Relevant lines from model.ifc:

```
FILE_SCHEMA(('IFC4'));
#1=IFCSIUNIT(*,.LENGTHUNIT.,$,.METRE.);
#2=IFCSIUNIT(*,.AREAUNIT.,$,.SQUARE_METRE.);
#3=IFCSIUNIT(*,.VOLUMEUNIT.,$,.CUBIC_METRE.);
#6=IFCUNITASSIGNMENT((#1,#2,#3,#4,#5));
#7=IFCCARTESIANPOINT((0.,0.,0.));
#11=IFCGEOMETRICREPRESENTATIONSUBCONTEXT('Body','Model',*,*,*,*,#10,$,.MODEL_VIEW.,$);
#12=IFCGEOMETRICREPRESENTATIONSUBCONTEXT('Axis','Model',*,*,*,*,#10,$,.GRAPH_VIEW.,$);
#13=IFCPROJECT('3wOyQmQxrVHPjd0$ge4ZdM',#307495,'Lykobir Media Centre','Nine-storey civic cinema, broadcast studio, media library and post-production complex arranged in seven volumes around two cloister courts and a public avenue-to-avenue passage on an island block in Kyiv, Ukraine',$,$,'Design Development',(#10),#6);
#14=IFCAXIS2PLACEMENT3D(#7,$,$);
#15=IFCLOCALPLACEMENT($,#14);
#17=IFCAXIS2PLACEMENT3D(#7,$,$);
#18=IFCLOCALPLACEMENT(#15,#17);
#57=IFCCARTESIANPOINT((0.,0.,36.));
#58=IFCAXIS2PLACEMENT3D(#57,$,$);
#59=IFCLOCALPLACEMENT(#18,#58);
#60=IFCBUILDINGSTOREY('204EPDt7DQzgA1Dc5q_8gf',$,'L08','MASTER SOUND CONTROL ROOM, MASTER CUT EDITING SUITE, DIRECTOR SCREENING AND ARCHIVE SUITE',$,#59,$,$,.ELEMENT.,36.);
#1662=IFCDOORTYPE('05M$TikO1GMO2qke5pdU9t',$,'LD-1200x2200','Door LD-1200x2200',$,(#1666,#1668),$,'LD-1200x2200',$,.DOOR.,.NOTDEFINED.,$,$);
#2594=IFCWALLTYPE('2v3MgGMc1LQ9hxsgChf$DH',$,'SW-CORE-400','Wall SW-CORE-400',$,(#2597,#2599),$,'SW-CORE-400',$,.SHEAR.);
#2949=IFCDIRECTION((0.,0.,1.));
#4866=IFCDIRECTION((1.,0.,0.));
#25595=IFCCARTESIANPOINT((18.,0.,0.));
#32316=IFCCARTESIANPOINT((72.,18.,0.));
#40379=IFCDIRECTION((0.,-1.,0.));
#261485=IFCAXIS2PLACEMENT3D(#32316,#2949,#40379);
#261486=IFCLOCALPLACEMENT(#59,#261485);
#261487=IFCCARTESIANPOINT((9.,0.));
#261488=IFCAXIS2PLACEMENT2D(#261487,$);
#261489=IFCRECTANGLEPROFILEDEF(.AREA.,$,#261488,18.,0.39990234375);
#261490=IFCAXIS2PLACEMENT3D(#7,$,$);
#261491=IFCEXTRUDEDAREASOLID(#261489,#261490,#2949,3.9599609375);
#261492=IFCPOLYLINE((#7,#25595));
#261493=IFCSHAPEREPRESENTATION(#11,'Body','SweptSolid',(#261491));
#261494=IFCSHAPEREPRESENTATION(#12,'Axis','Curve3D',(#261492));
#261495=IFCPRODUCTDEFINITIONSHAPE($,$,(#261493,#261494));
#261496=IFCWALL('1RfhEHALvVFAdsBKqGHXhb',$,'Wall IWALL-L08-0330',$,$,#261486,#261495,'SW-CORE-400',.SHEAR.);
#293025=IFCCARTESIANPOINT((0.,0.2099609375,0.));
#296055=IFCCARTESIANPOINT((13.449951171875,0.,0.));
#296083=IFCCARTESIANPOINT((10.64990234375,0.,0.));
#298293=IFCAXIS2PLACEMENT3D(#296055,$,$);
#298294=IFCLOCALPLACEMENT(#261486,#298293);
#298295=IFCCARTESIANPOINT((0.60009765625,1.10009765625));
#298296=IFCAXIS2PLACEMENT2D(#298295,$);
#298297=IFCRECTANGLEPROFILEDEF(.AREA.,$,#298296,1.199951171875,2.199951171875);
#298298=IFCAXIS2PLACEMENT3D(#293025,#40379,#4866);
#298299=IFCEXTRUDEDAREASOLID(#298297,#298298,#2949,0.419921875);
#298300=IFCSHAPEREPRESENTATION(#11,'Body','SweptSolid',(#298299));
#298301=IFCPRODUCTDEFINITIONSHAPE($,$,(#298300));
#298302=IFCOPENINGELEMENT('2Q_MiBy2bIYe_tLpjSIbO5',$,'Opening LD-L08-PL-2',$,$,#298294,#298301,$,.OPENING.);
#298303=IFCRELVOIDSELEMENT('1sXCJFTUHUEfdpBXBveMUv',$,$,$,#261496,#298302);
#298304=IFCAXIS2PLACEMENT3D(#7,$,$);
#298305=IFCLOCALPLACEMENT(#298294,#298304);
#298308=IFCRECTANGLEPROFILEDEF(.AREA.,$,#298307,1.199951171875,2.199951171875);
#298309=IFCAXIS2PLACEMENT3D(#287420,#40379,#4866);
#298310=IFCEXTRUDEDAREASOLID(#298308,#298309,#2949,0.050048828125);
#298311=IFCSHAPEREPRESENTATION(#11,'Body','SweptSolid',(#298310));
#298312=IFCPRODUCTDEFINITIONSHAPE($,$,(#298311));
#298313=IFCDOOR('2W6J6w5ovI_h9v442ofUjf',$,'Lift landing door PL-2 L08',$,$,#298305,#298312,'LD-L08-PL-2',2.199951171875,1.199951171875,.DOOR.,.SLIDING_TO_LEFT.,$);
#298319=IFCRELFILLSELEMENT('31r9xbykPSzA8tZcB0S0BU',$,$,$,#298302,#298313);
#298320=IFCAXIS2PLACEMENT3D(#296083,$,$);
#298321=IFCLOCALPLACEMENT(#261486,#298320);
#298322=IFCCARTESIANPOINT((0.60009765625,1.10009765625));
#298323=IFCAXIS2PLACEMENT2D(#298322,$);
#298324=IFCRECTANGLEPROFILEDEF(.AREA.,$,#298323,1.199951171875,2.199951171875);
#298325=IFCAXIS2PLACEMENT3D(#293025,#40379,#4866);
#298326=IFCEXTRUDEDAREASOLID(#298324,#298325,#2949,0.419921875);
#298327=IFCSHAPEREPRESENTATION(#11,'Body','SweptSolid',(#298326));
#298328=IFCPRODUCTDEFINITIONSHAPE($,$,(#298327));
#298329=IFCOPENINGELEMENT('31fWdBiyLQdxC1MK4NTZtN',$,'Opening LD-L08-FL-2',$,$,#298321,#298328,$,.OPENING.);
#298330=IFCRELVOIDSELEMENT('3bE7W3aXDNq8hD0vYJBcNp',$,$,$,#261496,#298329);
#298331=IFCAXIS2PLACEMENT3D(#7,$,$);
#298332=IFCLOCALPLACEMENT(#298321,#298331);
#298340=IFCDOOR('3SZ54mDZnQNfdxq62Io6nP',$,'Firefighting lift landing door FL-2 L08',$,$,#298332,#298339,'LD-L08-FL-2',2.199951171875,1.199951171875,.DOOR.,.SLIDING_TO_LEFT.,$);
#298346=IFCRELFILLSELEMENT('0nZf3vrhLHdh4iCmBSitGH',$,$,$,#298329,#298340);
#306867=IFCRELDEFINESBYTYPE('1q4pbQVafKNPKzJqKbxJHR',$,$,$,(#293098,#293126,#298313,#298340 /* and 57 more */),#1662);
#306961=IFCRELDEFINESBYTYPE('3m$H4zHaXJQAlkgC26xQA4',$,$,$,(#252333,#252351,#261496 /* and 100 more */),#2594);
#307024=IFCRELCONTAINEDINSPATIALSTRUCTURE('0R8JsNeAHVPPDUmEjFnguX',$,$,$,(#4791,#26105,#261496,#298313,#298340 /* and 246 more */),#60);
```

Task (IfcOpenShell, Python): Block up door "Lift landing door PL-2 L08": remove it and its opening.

```python
import ifcopenshell
import ifcopenshell.api.feature
import ifcopenshell.api.root
import ifcopenshell.geom
import ifcopenshell.util.shape

model = ifcopenshell.open("model.ifc")
settings = ifcopenshell.geom.settings()


def volume(element):
    """Net volume in cubic metres, openings subtracted."""
    shape = ifcopenshell.geom.create_shape(settings, element)
    return ifcopenshell.util.shape.get_volume(shape.geometry)


door = model.by_guid("2W6J6w5ovI_h9v442ofUjf")
opening = door.FillsVoids[0].RelatingOpeningElement
wall = opening.VoidsElements[0].RelatingBuildingElement
before = volume(wall)

ifcopenshell.api.root.remove_product(model, product=door)
ifcopenshell.api.feature.remove_feature(model, feature=opening)

after = volume(wall)

print(f"wall volume {before:.3f} -> {after:.3f} m3")

model.write("model_v2.ifc")
```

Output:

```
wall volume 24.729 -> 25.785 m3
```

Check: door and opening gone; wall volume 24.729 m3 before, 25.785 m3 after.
